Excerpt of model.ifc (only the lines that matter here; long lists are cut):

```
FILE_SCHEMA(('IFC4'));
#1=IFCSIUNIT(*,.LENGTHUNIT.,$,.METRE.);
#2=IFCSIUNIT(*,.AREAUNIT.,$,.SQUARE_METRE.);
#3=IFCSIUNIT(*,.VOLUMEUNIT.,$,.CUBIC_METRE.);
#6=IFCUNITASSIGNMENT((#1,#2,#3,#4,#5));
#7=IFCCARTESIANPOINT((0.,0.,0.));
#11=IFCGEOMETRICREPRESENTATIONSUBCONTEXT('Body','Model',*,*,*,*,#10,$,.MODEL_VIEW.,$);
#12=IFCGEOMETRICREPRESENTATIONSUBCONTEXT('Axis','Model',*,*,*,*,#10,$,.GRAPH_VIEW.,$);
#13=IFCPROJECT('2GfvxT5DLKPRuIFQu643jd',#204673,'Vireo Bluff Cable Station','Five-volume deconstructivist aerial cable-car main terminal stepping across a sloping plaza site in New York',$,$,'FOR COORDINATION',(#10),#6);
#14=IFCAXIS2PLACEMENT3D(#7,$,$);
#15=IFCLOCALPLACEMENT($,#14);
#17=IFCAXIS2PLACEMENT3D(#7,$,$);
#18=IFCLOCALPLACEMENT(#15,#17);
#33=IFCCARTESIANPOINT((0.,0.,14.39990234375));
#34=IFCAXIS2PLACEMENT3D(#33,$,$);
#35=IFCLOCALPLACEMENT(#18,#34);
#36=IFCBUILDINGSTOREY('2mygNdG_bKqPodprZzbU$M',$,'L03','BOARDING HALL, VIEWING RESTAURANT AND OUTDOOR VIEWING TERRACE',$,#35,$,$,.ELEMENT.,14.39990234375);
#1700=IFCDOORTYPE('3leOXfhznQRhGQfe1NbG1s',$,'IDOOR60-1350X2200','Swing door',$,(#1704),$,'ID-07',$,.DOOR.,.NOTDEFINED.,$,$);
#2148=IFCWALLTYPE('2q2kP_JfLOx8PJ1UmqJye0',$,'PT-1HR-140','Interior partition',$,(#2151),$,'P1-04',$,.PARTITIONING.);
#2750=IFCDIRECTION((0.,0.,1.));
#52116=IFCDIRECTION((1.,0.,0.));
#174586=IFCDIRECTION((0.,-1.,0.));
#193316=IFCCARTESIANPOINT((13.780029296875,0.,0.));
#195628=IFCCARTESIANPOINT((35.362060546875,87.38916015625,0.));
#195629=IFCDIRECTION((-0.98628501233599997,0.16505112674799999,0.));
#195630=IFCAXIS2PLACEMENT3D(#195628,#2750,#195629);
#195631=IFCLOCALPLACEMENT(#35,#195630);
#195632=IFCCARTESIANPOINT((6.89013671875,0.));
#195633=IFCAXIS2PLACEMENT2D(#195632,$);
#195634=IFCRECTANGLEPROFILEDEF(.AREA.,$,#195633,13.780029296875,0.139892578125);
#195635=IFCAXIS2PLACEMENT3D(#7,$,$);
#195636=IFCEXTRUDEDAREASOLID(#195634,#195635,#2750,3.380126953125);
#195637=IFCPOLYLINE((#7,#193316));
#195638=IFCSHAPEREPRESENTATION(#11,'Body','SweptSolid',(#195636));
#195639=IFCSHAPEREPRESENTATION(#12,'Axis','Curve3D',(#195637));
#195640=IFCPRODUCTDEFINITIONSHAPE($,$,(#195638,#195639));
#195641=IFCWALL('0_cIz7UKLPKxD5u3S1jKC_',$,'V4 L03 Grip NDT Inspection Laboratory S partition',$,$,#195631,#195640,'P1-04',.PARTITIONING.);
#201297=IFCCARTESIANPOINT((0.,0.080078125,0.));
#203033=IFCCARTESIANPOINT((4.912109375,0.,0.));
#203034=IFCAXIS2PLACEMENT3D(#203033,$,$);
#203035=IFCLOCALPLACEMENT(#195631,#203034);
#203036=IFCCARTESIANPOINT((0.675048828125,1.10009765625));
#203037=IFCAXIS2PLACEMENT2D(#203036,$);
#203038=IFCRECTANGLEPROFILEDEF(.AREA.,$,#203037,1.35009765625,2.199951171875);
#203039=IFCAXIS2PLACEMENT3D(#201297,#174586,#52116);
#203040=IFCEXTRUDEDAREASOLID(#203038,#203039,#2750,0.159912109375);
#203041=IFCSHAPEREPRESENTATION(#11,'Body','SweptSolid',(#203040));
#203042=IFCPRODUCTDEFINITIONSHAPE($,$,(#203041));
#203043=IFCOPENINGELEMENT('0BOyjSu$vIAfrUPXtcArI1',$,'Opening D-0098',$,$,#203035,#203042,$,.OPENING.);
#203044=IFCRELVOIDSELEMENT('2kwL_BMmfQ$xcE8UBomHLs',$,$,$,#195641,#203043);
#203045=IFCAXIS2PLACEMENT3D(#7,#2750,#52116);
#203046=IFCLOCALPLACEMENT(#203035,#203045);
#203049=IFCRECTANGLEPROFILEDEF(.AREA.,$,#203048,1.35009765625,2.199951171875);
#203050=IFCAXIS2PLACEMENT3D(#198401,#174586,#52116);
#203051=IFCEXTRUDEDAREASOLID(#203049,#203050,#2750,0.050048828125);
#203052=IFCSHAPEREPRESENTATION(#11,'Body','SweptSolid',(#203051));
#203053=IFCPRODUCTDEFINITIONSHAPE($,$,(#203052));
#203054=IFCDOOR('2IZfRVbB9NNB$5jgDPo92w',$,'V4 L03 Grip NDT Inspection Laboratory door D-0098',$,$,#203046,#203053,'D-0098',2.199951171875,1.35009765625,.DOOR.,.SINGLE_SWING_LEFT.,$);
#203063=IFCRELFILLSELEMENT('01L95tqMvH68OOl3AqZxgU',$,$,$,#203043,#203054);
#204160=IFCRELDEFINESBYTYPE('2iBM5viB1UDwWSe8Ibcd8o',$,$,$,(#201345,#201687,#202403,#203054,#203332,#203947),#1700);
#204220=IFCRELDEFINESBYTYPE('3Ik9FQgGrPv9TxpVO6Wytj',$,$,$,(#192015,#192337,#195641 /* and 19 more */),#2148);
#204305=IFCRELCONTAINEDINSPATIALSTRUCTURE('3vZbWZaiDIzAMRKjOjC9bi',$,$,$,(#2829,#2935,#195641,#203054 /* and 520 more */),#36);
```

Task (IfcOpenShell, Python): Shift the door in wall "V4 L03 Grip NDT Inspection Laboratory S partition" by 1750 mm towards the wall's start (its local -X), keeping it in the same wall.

```python
import ifcopenshell
import ifcopenshell.api.geometry
import ifcopenshell.util.placement
import ifcopenshell.util.unit

model = ifcopenshell.open("model.ifc")
unit_scale = ifcopenshell.util.unit.calculate_unit_scale(model)

door = model.by_guid("2IZfRVbB9NNB$5jgDPo92w")
opening = door.FillsVoids[0].RelatingOpeningElement
wall = opening.VoidsElements[0].RelatingBuildingElement

wall_matrix = ifcopenshell.util.placement.get_local_placement(wall.ObjectPlacement)
shift = wall_matrix[:3, 0] * -1.75 / unit_scale
before = ifcopenshell.util.placement.get_local_placement(door.ObjectPlacement)[:3, 3].copy()

# The door is placed relative to its opening, so it follows when the opening moves.
matrix = ifcopenshell.util.placement.get_local_placement(opening.ObjectPlacement)
matrix[:3, 3] += shift
ifcopenshell.api.geometry.edit_object_placement(
    model, product=opening, matrix=matrix, is_si=False, should_transform_children=True
)

after = ifcopenshell.util.placement.get_local_placement(door.ObjectPlacement)[:3, 3]
print("door moved by", (after - before).round(3) + 0.0)

model.write("model_updated.ifc")
```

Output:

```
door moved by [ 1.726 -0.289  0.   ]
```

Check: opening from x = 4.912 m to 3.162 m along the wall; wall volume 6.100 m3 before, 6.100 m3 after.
